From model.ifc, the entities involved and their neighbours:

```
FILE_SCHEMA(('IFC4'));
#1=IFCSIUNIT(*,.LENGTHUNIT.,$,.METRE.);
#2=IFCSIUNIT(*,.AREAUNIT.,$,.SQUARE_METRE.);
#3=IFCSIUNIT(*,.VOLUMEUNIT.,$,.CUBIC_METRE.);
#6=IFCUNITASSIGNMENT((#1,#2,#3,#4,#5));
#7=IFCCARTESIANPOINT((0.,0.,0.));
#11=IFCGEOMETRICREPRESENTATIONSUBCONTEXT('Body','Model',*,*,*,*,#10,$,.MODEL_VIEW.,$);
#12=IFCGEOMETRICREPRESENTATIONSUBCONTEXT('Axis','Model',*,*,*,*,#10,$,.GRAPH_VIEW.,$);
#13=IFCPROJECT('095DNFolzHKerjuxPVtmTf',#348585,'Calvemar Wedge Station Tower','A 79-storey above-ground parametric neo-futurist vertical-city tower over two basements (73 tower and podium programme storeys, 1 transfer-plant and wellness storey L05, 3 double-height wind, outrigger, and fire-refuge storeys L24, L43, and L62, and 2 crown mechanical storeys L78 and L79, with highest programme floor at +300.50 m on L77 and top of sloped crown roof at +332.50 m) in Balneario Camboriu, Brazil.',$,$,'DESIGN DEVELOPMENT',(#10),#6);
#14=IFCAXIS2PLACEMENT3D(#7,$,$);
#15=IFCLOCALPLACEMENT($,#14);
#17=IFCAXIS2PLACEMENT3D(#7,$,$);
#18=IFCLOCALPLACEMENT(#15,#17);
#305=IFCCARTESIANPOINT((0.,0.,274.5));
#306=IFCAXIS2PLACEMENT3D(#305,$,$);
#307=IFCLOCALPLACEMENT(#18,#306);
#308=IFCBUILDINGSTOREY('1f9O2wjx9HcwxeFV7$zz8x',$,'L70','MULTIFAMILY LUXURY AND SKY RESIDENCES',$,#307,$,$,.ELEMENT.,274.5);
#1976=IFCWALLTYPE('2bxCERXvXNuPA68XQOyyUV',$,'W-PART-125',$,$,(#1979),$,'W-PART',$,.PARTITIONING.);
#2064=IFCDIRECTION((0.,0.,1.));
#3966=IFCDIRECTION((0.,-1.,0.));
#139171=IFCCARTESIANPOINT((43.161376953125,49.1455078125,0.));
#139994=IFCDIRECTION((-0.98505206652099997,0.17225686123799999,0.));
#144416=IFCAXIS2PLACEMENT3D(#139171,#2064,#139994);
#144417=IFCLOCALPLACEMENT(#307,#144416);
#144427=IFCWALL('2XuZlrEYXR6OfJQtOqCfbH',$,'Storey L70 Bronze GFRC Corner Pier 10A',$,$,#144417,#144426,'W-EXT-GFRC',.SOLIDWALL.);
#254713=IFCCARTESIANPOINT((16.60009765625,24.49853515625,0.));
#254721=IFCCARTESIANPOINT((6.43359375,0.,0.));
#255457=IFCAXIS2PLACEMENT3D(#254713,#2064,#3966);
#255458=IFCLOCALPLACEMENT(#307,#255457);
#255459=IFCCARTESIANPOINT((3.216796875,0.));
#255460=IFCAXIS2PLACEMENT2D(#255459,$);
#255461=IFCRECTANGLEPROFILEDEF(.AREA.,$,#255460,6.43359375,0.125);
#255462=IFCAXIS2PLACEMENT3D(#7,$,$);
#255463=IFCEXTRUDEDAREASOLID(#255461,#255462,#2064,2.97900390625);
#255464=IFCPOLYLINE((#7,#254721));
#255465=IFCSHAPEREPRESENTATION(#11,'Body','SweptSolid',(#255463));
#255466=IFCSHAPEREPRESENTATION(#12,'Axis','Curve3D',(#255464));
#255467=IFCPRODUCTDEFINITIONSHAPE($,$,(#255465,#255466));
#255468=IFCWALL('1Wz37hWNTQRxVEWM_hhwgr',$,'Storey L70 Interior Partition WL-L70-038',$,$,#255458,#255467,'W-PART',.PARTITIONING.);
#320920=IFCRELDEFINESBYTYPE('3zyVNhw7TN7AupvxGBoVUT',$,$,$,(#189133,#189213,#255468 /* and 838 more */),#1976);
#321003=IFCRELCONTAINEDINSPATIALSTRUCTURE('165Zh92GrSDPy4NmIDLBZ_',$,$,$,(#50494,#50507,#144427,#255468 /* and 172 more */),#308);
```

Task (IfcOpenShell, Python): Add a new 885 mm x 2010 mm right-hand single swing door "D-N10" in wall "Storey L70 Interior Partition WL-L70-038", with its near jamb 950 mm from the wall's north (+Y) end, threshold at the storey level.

```python
import numpy as np
import ifcopenshell
import ifcopenshell.api.feature
import ifcopenshell.api.geometry
import ifcopenshell.api.root
import ifcopenshell.api.spatial
import ifcopenshell.geom
import ifcopenshell.util.element
import ifcopenshell.util.placement
import ifcopenshell.util.representation
import ifcopenshell.util.shape
import ifcopenshell.util.unit

model = ifcopenshell.open("model.ifc")
unit_scale = ifcopenshell.util.unit.calculate_unit_scale(model)
settings = ifcopenshell.geom.settings()


def volume(element):
    """Net volume in cubic metres, openings subtracted."""
    shape = ifcopenshell.geom.create_shape(settings, element)
    return ifcopenshell.util.shape.get_volume(shape.geometry)


wall = model.by_id(255468)
storey = ifcopenshell.util.element.get_container(wall, ifc_class="IfcBuildingStorey")
context = ifcopenshell.util.representation.get_context(model, "Model", "Body", "MODEL_VIEW")
before = volume(wall)

width, height, from_end, sill = 0.885, 2.01, 0.95, 0.0  # metres

# The wall runs along its own X axis, and the end named is its -X end.
wall_shape = ifcopenshell.geom.create_shape(settings, wall)
x, y, z = ifcopenshell.util.shape.get_vertices(wall_shape.geometry).T
start = x.min() + from_end
face, thickness = float(y.min()), float(y.max() - y.min())
wall_matrix = ifcopenshell.util.placement.get_local_placement(wall.ObjectPlacement)
level = ifcopenshell.util.placement.get_local_placement(storey.ObjectPlacement)[2, 3]


def in_wall(x, y):
    """Placement at x, y metres in the wall's axes, at sill height."""
    matrix = wall_matrix.copy()
    matrix[:, 3] = wall_matrix @ np.array([x / unit_scale, y / unit_scale, 0.0, 1.0])
    matrix[2, 3] = level + sill / unit_scale
    return matrix


# Opening: a box that overshoots both wall faces by 50 mm.
opening = ifcopenshell.api.root.create_entity(model, ifc_class="IfcOpeningElement", predefined_type="OPENING")
box = ifcopenshell.api.geometry.add_wall_representation(
    model, context=context, length=width, height=height, thickness=thickness + 0.1
)
ifcopenshell.api.geometry.assign_representation(model, product=opening, representation=box)
ifcopenshell.api.geometry.edit_object_placement(model, product=opening, matrix=in_wall(start, face - 0.05), is_si=False)
ifcopenshell.api.feature.add_feature(model, feature=opening, element=wall)

door = ifcopenshell.api.root.create_entity(model, ifc_class="IfcDoor", name="D-N10", predefined_type="DOOR")
door.OverallWidth, door.OverallHeight = width / unit_scale, height / unit_scale
door.OperationType = "SINGLE_SWING_RIGHT"
body = ifcopenshell.api.geometry.add_door_representation(
    model,
    context=context,
    overall_width=door.OverallWidth,
    overall_height=door.OverallHeight,
    operation_type="SINGLE_SWING_RIGHT",
    lining_properties={"LiningDepth": thickness / unit_scale, "ThresholdDepth": thickness / unit_scale},
)
ifcopenshell.api.geometry.assign_representation(model, product=door, representation=body)
ifcopenshell.api.spatial.assign_container(model, products=[door], relating_structure=storey)
ifcopenshell.api.feature.add_filling(model, opening=opening, element=door)

# The lining spans the wall, so the door starts at the wall face.
ifcopenshell.api.geometry.edit_object_placement(model, product=door, matrix=in_wall(start, face), is_si=False)

after = volume(wall)

print(f"wall volume {before:.3f} -> {after:.3f} m3")

model.write("model-out.ifc")
```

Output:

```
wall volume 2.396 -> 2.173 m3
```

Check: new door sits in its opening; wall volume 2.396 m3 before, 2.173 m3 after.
